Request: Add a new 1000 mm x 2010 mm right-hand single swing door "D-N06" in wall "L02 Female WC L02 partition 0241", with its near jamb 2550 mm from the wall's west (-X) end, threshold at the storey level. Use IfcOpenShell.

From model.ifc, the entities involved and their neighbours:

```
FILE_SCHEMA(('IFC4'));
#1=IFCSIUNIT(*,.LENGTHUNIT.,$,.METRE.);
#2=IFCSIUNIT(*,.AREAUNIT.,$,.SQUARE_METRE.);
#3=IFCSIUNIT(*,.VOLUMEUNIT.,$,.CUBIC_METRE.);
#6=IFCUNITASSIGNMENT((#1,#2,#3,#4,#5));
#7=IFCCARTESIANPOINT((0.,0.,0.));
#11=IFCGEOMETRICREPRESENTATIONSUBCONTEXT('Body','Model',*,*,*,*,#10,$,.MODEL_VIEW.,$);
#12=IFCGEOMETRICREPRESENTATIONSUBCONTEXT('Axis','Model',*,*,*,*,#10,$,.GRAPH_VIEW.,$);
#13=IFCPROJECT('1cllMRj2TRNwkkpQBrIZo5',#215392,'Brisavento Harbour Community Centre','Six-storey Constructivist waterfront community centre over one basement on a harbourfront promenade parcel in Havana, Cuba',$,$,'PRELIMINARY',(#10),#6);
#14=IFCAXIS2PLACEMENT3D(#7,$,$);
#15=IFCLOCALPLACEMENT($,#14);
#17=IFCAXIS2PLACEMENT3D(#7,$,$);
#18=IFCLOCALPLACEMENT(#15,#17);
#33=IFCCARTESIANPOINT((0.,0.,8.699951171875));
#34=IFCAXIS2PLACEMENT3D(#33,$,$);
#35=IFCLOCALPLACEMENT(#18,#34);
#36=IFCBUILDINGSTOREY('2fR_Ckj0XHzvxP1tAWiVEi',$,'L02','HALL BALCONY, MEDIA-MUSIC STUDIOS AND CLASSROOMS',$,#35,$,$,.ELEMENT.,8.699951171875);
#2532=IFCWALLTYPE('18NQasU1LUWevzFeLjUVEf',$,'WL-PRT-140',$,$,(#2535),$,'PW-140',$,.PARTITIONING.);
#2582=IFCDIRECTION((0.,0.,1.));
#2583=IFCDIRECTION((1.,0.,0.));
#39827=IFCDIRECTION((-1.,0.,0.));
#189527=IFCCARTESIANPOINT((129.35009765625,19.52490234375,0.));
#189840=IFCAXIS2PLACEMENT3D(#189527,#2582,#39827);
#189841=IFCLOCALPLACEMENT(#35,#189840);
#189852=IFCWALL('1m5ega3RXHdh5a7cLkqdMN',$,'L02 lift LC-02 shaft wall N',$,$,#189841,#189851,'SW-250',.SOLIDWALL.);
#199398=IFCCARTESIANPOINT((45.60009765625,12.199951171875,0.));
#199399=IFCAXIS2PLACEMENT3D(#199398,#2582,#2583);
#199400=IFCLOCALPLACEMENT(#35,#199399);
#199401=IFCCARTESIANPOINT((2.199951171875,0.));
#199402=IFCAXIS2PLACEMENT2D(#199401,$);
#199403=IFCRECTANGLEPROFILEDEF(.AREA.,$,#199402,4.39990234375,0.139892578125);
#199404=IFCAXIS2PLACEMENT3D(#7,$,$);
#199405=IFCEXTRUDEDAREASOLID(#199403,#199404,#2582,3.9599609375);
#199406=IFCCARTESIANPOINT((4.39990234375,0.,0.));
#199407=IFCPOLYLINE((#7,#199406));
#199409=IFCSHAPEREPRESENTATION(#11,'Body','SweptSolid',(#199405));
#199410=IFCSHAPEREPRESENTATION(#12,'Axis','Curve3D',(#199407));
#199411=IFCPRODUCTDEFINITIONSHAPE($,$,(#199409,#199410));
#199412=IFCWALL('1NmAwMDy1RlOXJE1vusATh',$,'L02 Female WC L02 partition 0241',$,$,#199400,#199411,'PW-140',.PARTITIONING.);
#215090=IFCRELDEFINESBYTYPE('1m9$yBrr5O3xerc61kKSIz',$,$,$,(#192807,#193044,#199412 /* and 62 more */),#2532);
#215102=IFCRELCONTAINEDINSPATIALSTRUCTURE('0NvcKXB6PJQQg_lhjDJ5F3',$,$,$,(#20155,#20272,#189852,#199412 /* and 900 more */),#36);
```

```python
import numpy as np
import ifcopenshell
import ifcopenshell.api.feature
import ifcopenshell.api.geometry
import ifcopenshell.api.root
import ifcopenshell.api.spatial
import ifcopenshell.geom
import ifcopenshell.util.element
import ifcopenshell.util.placement
import ifcopenshell.util.representation
import ifcopenshell.util.shape
import ifcopenshell.util.unit

model = ifcopenshell.open("model.ifc")
unit_scale = ifcopenshell.util.unit.calculate_unit_scale(model)
settings = ifcopenshell.geom.settings()


def volume(element):
    """Net volume in cubic metres, openings subtracted."""
    shape = ifcopenshell.geom.create_shape(settings, element)
    return ifcopenshell.util.shape.get_volume(shape.geometry)


wall = model.by_guid("1NmAwMDy1RlOXJE1vusATh")
storey = ifcopenshell.util.element.get_container(wall, ifc_class="IfcBuildingStorey")
context = ifcopenshell.util.representation.get_context(model, "Model", "Body", "MODEL_VIEW")
before = volume(wall)

width, height, from_end, sill = 1, 2.01, 2.55, 0.0  # metres

# The wall runs along its own X axis, and the end named is its -X end.
wall_shape = ifcopenshell.geom.create_shape(settings, wall)
x, y, z = ifcopenshell.util.shape.get_vertices(wall_shape.geometry).T
start = x.min() + from_end
face, thickness = float(y.min()), float(y.max() - y.min())
wall_matrix = ifcopenshell.util.placement.get_local_placement(wall.ObjectPlacement)
level = ifcopenshell.util.placement.get_local_placement(storey.ObjectPlacement)[2, 3]


def in_wall(x, y):
    """Placement at x, y metres in the wall's axes, at sill height."""
    matrix = wall_matrix.copy()
    matrix[:, 3] = wall_matrix @ np.array([x / unit_scale, y / unit_scale, 0.0, 1.0])
    matrix[2, 3] = level + sill / unit_scale
    return matrix


# Opening: a box that overshoots both wall faces by 50 mm.
opening = ifcopenshell.api.root.create_entity(model, ifc_class="IfcOpeningElement", predefined_type="OPENING")
box = ifcopenshell.api.geometry.add_wall_representation(
    model, context=context, length=width, height=height, thickness=thickness + 0.1
)
ifcopenshell.api.geometry.assign_representation(model, product=opening, representation=box)
ifcopenshell.api.geometry.edit_object_placement(model, product=opening, matrix=in_wall(start, face - 0.05), is_si=False)
ifcopenshell.api.feature.add_feature(model, feature=opening, element=wall)

door = ifcopenshell.api.root.create_entity(model, ifc_class="IfcDoor", name="D-N06", predefined_type="DOOR")
door.OverallWidth, door.OverallHeight = width / unit_scale, height / unit_scale
door.OperationType = "SINGLE_SWING_RIGHT"
body = ifcopenshell.api.geometry.add_door_representation(
    model,
    context=context,
    overall_width=door.OverallWidth,
    overall_height=door.OverallHeight,
    operation_type="SINGLE_SWING_RIGHT",
    lining_properties={"LiningDepth": thickness / unit_scale, "ThresholdDepth": thickness / unit_scale},
)
ifcopenshell.api.geometry.assign_representation(model, product=door, representation=body)
ifcopenshell.api.spatial.assign_container(model, products=[door], relating_structure=storey)
ifcopenshell.api.feature.add_filling(model, opening=opening, element=door)

# The lining spans the wall, so the door starts at the wall face.
ifcopenshell.api.geometry.edit_object_placement(model, product=door, matrix=in_wall(start, face), is_si=False)

after = volume(wall)

print(f"wall volume {before:.3f} -> {after:.3f} m3")

model.write("model-out.ifc")
```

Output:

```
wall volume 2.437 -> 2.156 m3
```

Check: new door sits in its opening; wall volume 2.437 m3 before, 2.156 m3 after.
